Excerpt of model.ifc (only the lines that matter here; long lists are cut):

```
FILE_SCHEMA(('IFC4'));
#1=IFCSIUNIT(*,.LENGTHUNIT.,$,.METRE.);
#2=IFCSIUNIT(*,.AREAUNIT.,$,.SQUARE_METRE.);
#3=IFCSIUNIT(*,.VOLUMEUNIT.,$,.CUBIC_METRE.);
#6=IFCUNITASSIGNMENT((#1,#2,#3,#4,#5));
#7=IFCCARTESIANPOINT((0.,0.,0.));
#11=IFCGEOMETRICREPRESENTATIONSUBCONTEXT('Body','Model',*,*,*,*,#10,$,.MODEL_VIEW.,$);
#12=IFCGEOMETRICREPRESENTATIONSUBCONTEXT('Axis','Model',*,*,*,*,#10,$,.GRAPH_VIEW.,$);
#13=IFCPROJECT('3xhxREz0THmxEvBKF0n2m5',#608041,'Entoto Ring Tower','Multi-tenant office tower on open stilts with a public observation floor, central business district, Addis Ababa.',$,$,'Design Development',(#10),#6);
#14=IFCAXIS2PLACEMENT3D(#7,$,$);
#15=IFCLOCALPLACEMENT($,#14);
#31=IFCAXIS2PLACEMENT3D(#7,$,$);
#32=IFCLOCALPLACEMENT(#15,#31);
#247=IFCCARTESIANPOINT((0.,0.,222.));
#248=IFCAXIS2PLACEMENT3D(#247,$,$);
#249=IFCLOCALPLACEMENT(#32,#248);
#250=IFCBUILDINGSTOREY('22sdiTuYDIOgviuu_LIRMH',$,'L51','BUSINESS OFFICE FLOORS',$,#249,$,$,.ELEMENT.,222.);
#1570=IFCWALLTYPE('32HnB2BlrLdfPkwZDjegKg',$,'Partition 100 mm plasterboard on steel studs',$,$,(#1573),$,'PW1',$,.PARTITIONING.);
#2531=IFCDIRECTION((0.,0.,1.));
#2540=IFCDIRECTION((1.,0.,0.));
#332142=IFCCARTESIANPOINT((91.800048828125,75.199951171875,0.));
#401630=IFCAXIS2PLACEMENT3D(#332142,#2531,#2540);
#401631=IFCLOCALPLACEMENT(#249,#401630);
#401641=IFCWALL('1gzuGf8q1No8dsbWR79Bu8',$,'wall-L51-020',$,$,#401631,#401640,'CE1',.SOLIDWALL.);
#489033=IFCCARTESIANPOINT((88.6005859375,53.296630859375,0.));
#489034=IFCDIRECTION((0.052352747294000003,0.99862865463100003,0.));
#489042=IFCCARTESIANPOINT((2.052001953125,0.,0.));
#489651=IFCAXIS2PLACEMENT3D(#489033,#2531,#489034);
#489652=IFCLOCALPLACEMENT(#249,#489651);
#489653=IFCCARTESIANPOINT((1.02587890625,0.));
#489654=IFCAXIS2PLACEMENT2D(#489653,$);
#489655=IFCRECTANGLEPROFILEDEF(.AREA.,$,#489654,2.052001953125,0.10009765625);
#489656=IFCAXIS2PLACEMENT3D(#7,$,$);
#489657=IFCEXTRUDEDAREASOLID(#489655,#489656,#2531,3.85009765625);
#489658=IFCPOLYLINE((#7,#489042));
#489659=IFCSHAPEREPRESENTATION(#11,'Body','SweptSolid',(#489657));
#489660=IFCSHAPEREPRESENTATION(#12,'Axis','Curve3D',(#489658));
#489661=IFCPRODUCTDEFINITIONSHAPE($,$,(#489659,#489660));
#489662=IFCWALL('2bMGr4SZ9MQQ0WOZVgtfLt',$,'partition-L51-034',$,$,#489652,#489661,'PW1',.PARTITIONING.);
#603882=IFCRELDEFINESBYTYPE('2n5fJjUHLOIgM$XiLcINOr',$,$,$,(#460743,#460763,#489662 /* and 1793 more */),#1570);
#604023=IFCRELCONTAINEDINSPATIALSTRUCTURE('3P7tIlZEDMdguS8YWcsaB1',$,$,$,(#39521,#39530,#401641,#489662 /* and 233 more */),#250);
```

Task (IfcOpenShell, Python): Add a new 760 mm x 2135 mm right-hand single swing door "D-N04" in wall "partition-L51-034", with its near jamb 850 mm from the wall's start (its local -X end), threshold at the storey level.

```python
import numpy as np
import ifcopenshell
import ifcopenshell.api.feature
import ifcopenshell.api.geometry
import ifcopenshell.api.root
import ifcopenshell.api.spatial
import ifcopenshell.geom
import ifcopenshell.util.element
import ifcopenshell.util.placement
import ifcopenshell.util.representation
import ifcopenshell.util.shape
import ifcopenshell.util.unit

model = ifcopenshell.open("model.ifc")
unit_scale = ifcopenshell.util.unit.calculate_unit_scale(model)
settings = ifcopenshell.geom.settings()


def volume(element):
    """Net volume in cubic metres, openings subtracted."""
    shape = ifcopenshell.geom.create_shape(settings, element)
    return ifcopenshell.util.shape.get_volume(shape.geometry)


wall = model.by_id(489662)
storey = ifcopenshell.util.element.get_container(wall, ifc_class="IfcBuildingStorey")
context = ifcopenshell.util.representation.get_context(model, "Model", "Body", "MODEL_VIEW")
before = volume(wall)

width, height, from_end, sill = 0.76, 2.135, 0.85, 0.0  # metres

# The wall runs along its own X axis, and the end named is its -X end.
wall_shape = ifcopenshell.geom.create_shape(settings, wall)
x, y, z = ifcopenshell.util.shape.get_vertices(wall_shape.geometry).T
start = x.min() + from_end
face, thickness = float(y.min()), float(y.max() - y.min())
wall_matrix = ifcopenshell.util.placement.get_local_placement(wall.ObjectPlacement)
level = ifcopenshell.util.placement.get_local_placement(storey.ObjectPlacement)[2, 3]


def in_wall(x, y):
    """Placement at x, y metres in the wall's axes, at sill height."""
    matrix = wall_matrix.copy()
    matrix[:, 3] = wall_matrix @ np.array([x / unit_scale, y / unit_scale, 0.0, 1.0])
    matrix[2, 3] = level + sill / unit_scale
    return matrix


# Opening: a box that overshoots both wall faces by 50 mm.
opening = ifcopenshell.api.root.create_entity(model, ifc_class="IfcOpeningElement", predefined_type="OPENING")
box = ifcopenshell.api.geometry.add_wall_representation(
    model, context=context, length=width, height=height, thickness=thickness + 0.1
)
ifcopenshell.api.geometry.assign_representation(model, product=opening, representation=box)
ifcopenshell.api.geometry.edit_object_placement(model, product=opening, matrix=in_wall(start, face - 0.05), is_si=False)
ifcopenshell.api.feature.add_feature(model, feature=opening, element=wall)

door = ifcopenshell.api.root.create_entity(model, ifc_class="IfcDoor", name="D-N04", predefined_type="DOOR")
door.OverallWidth, door.OverallHeight = width / unit_scale, height / unit_scale
door.OperationType = "SINGLE_SWING_RIGHT"
body = ifcopenshell.api.geometry.add_door_representation(
    model,
    context=context,
    overall_width=door.OverallWidth,
    overall_height=door.OverallHeight,
    operation_type="SINGLE_SWING_RIGHT",
    lining_properties={"LiningDepth": thickness / unit_scale, "ThresholdDepth": thickness / unit_scale},
)
ifcopenshell.api.geometry.assign_representation(model, product=door, representation=body)
ifcopenshell.api.spatial.assign_container(model, products=[door], relating_structure=storey)
ifcopenshell.api.feature.add_filling(model, opening=opening, element=door)

# The lining spans the wall, so the door starts at the wall face.
ifcopenshell.api.geometry.edit_object_placement(model, product=door, matrix=in_wall(start, face), is_si=False)

after = volume(wall)

print(f"wall volume {before:.3f} -> {after:.3f} m3")

model.write("model_updated.ifc")
```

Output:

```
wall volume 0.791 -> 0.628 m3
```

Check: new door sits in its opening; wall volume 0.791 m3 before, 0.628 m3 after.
